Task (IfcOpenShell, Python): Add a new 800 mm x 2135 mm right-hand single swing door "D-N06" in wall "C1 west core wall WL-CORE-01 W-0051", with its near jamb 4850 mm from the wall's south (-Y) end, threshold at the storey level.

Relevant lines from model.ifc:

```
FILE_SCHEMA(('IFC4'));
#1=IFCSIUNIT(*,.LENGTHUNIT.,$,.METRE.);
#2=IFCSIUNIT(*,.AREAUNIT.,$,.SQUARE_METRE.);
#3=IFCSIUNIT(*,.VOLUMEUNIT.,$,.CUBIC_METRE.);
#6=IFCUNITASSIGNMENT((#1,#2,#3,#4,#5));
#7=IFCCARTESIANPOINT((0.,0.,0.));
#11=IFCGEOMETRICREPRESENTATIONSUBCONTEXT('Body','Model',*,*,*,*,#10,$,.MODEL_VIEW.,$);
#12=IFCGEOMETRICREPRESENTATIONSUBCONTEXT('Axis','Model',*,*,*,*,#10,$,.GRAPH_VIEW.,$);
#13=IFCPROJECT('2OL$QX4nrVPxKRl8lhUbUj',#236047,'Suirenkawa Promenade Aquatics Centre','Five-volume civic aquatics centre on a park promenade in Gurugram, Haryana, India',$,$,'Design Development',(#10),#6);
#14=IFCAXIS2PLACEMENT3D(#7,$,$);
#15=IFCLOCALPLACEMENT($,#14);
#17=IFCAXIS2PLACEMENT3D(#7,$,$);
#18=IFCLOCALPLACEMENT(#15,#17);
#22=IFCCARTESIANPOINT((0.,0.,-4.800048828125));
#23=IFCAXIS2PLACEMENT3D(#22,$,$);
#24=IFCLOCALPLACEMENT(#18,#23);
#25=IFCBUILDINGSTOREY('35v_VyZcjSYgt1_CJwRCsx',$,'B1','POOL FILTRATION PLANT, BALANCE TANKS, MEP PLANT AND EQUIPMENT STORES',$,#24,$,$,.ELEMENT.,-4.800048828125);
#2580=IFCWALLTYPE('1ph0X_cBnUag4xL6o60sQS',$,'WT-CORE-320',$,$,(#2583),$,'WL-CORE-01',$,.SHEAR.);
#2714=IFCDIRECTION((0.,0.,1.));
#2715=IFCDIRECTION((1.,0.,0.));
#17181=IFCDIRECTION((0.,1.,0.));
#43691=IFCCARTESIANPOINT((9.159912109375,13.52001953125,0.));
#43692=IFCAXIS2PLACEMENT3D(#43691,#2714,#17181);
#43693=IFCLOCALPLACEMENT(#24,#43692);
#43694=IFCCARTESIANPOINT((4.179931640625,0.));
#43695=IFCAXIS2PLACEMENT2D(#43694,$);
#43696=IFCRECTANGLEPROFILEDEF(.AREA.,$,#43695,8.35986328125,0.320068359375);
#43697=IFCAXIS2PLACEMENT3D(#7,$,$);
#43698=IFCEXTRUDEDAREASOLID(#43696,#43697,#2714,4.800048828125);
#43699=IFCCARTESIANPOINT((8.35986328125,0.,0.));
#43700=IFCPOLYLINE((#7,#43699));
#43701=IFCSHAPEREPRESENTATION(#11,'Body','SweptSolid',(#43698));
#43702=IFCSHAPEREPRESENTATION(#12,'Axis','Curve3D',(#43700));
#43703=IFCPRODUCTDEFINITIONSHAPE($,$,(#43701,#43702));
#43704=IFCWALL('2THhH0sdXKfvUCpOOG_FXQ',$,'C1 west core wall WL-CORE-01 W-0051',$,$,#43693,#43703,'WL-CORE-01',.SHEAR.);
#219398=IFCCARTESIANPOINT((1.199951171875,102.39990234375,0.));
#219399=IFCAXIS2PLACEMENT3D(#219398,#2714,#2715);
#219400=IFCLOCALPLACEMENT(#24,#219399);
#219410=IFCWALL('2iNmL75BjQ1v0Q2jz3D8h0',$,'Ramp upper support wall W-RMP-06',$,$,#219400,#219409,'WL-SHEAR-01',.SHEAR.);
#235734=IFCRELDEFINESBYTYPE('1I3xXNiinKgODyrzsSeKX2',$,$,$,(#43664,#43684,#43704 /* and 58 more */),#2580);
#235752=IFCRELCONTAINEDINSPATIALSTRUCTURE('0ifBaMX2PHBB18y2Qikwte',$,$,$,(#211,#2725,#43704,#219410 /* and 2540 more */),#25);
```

```python
import numpy as np
import ifcopenshell
import ifcopenshell.api.feature
import ifcopenshell.api.geometry
import ifcopenshell.api.root
import ifcopenshell.api.spatial
import ifcopenshell.geom
import ifcopenshell.util.element
import ifcopenshell.util.placement
import ifcopenshell.util.representation
import ifcopenshell.util.shape
import ifcopenshell.util.unit

model = ifcopenshell.open("model.ifc")
unit_scale = ifcopenshell.util.unit.calculate_unit_scale(model)
settings = ifcopenshell.geom.settings()


def volume(element):
    """Net volume in cubic metres, openings subtracted."""
    shape = ifcopenshell.geom.create_shape(settings, element)
    return ifcopenshell.util.shape.get_volume(shape.geometry)


wall = model.by_guid("2THhH0sdXKfvUCpOOG_FXQ")
storey = ifcopenshell.util.element.get_container(wall, ifc_class="IfcBuildingStorey")
context = ifcopenshell.util.representation.get_context(model, "Model", "Body", "MODEL_VIEW")
before = volume(wall)

width, height, from_end, sill = 0.8, 2.135, 4.85, 0.0  # metres

# The wall runs along its own X axis, and the end named is its -X end.
wall_shape = ifcopenshell.geom.create_shape(settings, wall)
x, y, z = ifcopenshell.util.shape.get_vertices(wall_shape.geometry).T
start = x.min() + from_end
face, thickness = float(y.min()), float(y.max() - y.min())
wall_matrix = ifcopenshell.util.placement.get_local_placement(wall.ObjectPlacement)
level = ifcopenshell.util.placement.get_local_placement(storey.ObjectPlacement)[2, 3]


def in_wall(x, y):
    """Placement at x, y metres in the wall's axes, at sill height."""
    matrix = wall_matrix.copy()
    matrix[:, 3] = wall_matrix @ np.array([x / unit_scale, y / unit_scale, 0.0, 1.0])
    matrix[2, 3] = level + sill / unit_scale
    return matrix


# Opening: a box that overshoots both wall faces by 50 mm.
opening = ifcopenshell.api.root.create_entity(model, ifc_class="IfcOpeningElement", predefined_type="OPENING")
box = ifcopenshell.api.geometry.add_wall_representation(
    model, context=context, length=width, height=height, thickness=thickness + 0.1
)
ifcopenshell.api.geometry.assign_representation(model, product=opening, representation=box)
ifcopenshell.api.geometry.edit_object_placement(model, product=opening, matrix=in_wall(start, face - 0.05), is_si=False)
ifcopenshell.api.feature.add_feature(model, feature=opening, element=wall)

door = ifcopenshell.api.root.create_entity(model, ifc_class="IfcDoor", name="D-N06", predefined_type="DOOR")
door.OverallWidth, door.OverallHeight = width / unit_scale, height / unit_scale
door.OperationType = "SINGLE_SWING_RIGHT"
body = ifcopenshell.api.geometry.add_door_representation(
    model,
    context=context,
    overall_width=door.OverallWidth,
    overall_height=door.OverallHeight,
    operation_type="SINGLE_SWING_RIGHT",
    lining_properties={"LiningDepth": thickness / unit_scale, "ThresholdDepth": thickness / unit_scale},
)
ifcopenshell.api.geometry.assign_representation(model, product=door, representation=body)
ifcopenshell.api.spatial.assign_container(model, products=[door], relating_structure=storey)
ifcopenshell.api.feature.add_filling(model, opening=opening, element=door)

# The lining spans the wall, so the door starts at the wall face.
ifcopenshell.api.geometry.edit_object_placement(model, product=door, matrix=in_wall(start, face), is_si=False)

after = volume(wall)

print(f"wall volume {before:.3f} -> {after:.3f} m3")

model.write("model_v2.ifc")
```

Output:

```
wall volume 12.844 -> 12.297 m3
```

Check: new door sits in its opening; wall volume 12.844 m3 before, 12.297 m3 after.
